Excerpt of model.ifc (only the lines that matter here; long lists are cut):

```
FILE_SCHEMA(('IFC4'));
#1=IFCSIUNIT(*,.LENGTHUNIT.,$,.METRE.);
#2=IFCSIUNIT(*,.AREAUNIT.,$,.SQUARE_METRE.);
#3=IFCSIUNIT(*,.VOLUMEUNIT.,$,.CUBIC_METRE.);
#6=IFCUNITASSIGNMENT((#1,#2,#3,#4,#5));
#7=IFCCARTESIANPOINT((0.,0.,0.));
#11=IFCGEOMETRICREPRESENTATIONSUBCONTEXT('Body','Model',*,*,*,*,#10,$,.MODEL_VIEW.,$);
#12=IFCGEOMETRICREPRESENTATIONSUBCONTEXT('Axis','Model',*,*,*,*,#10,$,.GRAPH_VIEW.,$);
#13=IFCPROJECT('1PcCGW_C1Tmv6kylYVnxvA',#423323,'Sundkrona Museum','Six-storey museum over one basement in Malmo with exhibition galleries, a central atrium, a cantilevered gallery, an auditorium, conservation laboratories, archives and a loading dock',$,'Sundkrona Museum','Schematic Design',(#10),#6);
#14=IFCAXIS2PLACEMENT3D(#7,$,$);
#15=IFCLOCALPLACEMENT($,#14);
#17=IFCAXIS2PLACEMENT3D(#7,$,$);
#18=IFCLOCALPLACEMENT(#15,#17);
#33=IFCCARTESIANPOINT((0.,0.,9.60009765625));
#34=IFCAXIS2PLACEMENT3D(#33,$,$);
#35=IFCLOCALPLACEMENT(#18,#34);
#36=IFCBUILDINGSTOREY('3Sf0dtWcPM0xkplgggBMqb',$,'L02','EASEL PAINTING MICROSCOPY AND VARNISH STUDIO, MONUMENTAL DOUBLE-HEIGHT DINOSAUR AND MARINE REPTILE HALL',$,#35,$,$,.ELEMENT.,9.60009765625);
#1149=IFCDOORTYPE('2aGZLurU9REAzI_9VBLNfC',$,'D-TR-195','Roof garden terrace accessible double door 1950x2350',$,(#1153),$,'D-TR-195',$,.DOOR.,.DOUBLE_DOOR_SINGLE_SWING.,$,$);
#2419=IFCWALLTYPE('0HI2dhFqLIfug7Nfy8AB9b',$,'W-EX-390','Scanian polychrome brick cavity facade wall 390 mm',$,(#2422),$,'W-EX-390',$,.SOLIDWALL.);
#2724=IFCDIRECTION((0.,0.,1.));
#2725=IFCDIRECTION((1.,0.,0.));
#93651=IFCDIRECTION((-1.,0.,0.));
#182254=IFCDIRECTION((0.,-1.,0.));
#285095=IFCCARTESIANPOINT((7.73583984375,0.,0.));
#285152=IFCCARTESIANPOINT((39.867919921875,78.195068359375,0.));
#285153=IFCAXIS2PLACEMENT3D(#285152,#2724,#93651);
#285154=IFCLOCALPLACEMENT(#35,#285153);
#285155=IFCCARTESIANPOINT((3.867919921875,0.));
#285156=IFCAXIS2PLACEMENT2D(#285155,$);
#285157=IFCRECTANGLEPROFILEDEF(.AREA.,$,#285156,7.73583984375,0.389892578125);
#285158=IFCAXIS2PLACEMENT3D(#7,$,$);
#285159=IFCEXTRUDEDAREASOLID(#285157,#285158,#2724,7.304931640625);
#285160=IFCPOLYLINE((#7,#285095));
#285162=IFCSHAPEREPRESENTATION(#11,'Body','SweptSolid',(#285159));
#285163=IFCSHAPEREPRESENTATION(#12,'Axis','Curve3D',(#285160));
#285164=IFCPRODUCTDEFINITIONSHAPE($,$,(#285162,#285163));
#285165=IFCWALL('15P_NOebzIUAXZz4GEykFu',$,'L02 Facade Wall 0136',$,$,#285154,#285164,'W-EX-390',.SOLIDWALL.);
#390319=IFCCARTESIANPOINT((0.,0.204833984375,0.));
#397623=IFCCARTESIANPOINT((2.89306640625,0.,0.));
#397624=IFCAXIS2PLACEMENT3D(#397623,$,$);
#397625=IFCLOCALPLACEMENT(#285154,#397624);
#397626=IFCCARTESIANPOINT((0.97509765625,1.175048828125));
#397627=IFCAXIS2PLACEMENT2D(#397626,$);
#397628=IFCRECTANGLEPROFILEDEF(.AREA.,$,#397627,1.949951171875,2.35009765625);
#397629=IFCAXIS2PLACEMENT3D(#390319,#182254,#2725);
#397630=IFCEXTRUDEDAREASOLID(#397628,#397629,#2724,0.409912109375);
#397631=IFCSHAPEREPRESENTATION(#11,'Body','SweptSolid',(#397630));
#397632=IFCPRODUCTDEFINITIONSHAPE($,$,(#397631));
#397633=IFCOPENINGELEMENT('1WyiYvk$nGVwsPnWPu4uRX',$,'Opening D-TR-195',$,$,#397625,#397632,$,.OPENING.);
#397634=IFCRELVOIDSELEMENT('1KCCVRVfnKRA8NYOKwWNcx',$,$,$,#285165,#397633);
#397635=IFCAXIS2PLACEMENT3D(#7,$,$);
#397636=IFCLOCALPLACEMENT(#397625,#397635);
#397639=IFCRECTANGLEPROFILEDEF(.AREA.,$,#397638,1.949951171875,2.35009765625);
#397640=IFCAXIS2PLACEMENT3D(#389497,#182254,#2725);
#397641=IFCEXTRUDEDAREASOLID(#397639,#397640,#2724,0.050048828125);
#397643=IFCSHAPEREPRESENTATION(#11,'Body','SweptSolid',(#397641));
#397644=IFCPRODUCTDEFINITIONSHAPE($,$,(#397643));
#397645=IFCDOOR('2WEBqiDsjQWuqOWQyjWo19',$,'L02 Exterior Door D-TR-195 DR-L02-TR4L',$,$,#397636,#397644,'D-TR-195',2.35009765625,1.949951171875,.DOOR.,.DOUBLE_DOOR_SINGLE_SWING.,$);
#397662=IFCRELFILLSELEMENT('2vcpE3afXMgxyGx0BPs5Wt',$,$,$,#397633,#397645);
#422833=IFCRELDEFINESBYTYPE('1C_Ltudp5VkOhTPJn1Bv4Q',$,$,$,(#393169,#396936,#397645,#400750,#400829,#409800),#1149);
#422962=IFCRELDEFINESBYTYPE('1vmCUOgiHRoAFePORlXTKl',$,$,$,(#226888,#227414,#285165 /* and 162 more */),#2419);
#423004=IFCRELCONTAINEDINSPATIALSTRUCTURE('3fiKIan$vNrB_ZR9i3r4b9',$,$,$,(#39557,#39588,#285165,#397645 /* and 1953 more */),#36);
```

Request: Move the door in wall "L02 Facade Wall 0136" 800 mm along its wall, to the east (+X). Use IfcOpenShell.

```python
import ifcopenshell
import ifcopenshell.api.geometry
import ifcopenshell.util.placement
import ifcopenshell.util.unit

model = ifcopenshell.open("model.ifc")
unit_scale = ifcopenshell.util.unit.calculate_unit_scale(model)

door = model.by_guid("2WEBqiDsjQWuqOWQyjWo19")
opening = door.FillsVoids[0].RelatingOpeningElement
wall = opening.VoidsElements[0].RelatingBuildingElement

wall_matrix = ifcopenshell.util.placement.get_local_placement(wall.ObjectPlacement)
shift = wall_matrix[:3, 0] * -0.8 / unit_scale
before = ifcopenshell.util.placement.get_local_placement(door.ObjectPlacement)[:3, 3].copy()

# The door is placed relative to its opening, so it follows when the opening moves.
matrix = ifcopenshell.util.placement.get_local_placement(opening.ObjectPlacement)
matrix[:3, 3] += shift
ifcopenshell.api.geometry.edit_object_placement(
    model, product=opening, matrix=matrix, is_si=False, should_transform_children=True
)

after = ifcopenshell.util.placement.get_local_placement(door.ObjectPlacement)[:3, 3]
print("door moved by", (after - before).round(3) + 0.0)

model.write("model_rev.ifc")
```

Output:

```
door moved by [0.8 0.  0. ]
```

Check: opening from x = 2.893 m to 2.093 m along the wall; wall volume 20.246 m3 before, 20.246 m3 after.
